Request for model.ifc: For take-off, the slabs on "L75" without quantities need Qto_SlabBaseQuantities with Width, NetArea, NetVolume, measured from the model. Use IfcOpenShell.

First a look at what the model holds.

```python
import ifcopenshell
import ifcopenshell.util.element
import ifcopenshell.util.unit

model = ifcopenshell.open("model.ifc")
print(model.schema)
for unit_type in ("LENGTHUNIT", "AREAUNIT", "VOLUMEUNIT"):
    print(unit_type, ifcopenshell.util.unit.calculate_unit_scale(model, unit_type))
storey = next(s for s in model.by_type("IfcBuildingStorey") if s.Name == "L75")
slabs = [e for e in ifcopenshell.util.element.get_decomposition(storey) if e.is_a("IfcSlab")]
for e in sorted(slabs, key=lambda e: e.id()):
    print(e.id(), e.is_a(), e.Name, list(ifcopenshell.util.element.get_psets(e, qtos_only=True)), sep=" | ")
```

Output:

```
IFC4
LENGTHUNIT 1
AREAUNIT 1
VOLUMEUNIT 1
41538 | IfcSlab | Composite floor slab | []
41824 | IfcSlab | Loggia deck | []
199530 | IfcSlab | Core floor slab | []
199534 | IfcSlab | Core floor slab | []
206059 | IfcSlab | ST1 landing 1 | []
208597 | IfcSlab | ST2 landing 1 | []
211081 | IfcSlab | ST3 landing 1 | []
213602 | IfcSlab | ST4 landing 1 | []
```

```python
import ifcopenshell
import ifcopenshell.api.pset
import ifcopenshell.geom
import ifcopenshell.util.element
import ifcopenshell.util.shape
import ifcopenshell.util.unit

model = ifcopenshell.open("model.ifc")
unit_scale = ifcopenshell.util.unit.calculate_unit_scale(model)
area_scale = ifcopenshell.util.unit.calculate_unit_scale(model, "AREAUNIT")
volume_scale = ifcopenshell.util.unit.calculate_unit_scale(model, "VOLUMEUNIT")
settings = ifcopenshell.geom.settings()

storey = next(s for s in model.by_type("IfcBuildingStorey") if s.Name == "L75")
slabs = [e for e in ifcopenshell.util.element.get_decomposition(storey) if e.is_a("IfcSlab")]

for e in sorted(slabs, key=lambda e: e.id()):
    if ifcopenshell.util.element.get_psets(e, qtos_only=True, should_inherit=False):
        continue
    # Geometry comes back in metres, in the element's own axes.
    shape = ifcopenshell.geom.create_shape(settings, e)
    values = {
        "Width": ifcopenshell.util.shape.get_z(shape.geometry) / unit_scale,
        "NetArea": ifcopenshell.util.shape.get_footprint_area(shape.geometry) / area_scale,
        "NetVolume": ifcopenshell.util.shape.get_volume(shape.geometry) / volume_scale,
    }
    qto = ifcopenshell.api.pset.add_qto(model, product=e, name="Qto_SlabBaseQuantities")
    ifcopenshell.api.pset.edit_qto(model, qto=qto, properties=values)
    print(e.id(), {k: round(v, 3) for k, v in values.items()})

model.write("model_rev.ifc")
```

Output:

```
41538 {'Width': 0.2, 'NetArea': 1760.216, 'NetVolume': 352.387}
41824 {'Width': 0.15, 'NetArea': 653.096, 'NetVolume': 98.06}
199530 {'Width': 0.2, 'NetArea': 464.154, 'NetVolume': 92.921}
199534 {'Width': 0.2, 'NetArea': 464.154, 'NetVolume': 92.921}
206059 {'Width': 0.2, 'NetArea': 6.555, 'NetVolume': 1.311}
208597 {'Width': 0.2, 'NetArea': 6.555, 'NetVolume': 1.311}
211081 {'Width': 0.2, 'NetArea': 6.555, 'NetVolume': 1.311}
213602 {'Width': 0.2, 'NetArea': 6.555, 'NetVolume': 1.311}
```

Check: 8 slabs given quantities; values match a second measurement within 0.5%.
